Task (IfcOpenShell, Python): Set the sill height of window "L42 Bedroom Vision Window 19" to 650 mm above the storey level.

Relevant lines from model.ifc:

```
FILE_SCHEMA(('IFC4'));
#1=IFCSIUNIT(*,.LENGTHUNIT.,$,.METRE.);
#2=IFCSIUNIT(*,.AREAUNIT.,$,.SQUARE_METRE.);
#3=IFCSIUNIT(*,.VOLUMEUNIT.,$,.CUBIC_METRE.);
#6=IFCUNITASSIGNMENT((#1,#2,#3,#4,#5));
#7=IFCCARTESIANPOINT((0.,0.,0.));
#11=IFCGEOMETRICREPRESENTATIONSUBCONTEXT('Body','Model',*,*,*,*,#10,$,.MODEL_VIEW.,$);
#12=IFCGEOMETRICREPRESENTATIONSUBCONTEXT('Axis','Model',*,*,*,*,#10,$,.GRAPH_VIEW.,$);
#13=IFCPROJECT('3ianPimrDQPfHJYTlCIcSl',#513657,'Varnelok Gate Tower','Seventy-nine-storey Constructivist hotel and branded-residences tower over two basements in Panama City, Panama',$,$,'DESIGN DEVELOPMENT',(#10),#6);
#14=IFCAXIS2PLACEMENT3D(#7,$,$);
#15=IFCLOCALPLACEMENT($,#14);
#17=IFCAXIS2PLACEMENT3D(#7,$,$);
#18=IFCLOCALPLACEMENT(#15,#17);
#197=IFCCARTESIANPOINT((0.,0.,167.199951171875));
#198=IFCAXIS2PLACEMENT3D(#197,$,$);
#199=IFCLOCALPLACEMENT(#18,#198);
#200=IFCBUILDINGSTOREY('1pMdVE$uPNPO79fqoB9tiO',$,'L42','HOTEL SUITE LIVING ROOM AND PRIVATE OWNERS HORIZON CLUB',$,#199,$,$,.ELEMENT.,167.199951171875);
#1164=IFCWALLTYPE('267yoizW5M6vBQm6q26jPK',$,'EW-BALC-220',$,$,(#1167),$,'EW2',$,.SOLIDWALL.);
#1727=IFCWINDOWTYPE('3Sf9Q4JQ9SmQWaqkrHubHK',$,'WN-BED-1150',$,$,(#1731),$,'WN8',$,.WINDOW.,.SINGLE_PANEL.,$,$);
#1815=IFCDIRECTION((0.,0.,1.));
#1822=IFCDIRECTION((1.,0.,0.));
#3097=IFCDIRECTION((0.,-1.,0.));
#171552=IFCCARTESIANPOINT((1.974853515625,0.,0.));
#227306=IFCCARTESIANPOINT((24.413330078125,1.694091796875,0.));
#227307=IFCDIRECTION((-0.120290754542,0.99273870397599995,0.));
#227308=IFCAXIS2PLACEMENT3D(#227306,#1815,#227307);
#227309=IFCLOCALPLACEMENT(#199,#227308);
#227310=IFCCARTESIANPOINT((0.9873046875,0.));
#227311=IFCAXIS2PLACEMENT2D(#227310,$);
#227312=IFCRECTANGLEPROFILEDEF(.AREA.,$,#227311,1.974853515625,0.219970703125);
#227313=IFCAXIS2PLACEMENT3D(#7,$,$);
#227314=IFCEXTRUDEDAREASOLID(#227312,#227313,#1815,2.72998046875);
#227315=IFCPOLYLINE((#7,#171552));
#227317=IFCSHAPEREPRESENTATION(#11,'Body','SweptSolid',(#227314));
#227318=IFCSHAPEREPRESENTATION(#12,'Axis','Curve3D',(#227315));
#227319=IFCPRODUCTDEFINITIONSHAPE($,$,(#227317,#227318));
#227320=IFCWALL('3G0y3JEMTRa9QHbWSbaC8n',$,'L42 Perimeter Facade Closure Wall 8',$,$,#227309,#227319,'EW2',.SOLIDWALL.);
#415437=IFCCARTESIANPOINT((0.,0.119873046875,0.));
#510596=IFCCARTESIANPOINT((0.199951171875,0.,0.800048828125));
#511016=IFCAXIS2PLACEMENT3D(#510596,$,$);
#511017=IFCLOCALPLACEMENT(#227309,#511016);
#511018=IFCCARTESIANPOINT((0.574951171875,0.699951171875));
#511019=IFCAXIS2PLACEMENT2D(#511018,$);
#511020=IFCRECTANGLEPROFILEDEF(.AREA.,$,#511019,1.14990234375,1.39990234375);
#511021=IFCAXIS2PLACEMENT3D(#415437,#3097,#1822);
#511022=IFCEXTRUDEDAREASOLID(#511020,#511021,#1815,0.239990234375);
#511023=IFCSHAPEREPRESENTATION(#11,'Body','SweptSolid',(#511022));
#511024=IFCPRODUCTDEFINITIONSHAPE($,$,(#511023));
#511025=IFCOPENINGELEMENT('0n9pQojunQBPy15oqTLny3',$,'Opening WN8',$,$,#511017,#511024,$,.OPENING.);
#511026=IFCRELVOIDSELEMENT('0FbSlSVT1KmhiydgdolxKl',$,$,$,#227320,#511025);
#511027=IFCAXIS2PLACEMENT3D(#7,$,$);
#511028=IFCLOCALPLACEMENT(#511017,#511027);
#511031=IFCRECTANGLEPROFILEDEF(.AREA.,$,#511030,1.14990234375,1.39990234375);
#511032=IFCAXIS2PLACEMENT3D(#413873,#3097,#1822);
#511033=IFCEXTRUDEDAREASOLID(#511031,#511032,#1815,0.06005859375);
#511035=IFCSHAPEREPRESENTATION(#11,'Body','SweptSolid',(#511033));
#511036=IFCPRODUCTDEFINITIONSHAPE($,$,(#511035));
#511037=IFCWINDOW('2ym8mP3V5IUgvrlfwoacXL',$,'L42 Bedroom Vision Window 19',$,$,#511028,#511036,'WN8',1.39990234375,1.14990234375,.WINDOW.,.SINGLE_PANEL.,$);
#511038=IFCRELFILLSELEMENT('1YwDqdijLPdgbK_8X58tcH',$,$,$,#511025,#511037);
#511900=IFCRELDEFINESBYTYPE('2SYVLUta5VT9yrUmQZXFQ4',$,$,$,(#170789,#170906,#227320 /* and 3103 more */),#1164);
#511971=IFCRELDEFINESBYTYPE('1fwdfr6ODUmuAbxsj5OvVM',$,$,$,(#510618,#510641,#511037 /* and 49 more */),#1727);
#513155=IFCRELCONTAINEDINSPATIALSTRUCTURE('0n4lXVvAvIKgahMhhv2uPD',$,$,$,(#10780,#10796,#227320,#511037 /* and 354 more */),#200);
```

```python
import numpy as np
import ifcopenshell
import ifcopenshell.api.geometry
import ifcopenshell.geom
import ifcopenshell.util.element
import ifcopenshell.util.placement
import ifcopenshell.util.shape
import ifcopenshell.util.unit

model = ifcopenshell.open("model.ifc")
unit_scale = ifcopenshell.util.unit.calculate_unit_scale(model)

window = model.by_id(511037)
opening = window.FillsVoids[0].RelatingOpeningElement
storey = ifcopenshell.util.element.get_container(window, ifc_class="IfcBuildingStorey")
level = ifcopenshell.util.placement.get_local_placement(storey.ObjectPlacement)[2, 3]

# The opening's origin need not be at the sill, so measure its lowest point.
shape = ifcopenshell.geom.create_shape(ifcopenshell.geom.settings(), opening)
bottom = ifcopenshell.util.shape.get_shape_bottom_elevation(shape, shape.geometry) / unit_scale
dz = level + 0.65 / unit_scale - bottom

shift = np.array([0.0, 0.0, dz])
# The window is placed relative to its opening, so it follows when the opening moves.
matrix = ifcopenshell.util.placement.get_local_placement(opening.ObjectPlacement)
matrix[:3, 3] += shift
ifcopenshell.api.geometry.edit_object_placement(
    model, product=opening, matrix=matrix, is_si=False, should_transform_children=True
)

print(f"moved by {dz * unit_scale:+.3f} m")

model.write("model_updated.ifc")
```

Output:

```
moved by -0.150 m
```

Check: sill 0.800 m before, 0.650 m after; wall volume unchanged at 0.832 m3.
